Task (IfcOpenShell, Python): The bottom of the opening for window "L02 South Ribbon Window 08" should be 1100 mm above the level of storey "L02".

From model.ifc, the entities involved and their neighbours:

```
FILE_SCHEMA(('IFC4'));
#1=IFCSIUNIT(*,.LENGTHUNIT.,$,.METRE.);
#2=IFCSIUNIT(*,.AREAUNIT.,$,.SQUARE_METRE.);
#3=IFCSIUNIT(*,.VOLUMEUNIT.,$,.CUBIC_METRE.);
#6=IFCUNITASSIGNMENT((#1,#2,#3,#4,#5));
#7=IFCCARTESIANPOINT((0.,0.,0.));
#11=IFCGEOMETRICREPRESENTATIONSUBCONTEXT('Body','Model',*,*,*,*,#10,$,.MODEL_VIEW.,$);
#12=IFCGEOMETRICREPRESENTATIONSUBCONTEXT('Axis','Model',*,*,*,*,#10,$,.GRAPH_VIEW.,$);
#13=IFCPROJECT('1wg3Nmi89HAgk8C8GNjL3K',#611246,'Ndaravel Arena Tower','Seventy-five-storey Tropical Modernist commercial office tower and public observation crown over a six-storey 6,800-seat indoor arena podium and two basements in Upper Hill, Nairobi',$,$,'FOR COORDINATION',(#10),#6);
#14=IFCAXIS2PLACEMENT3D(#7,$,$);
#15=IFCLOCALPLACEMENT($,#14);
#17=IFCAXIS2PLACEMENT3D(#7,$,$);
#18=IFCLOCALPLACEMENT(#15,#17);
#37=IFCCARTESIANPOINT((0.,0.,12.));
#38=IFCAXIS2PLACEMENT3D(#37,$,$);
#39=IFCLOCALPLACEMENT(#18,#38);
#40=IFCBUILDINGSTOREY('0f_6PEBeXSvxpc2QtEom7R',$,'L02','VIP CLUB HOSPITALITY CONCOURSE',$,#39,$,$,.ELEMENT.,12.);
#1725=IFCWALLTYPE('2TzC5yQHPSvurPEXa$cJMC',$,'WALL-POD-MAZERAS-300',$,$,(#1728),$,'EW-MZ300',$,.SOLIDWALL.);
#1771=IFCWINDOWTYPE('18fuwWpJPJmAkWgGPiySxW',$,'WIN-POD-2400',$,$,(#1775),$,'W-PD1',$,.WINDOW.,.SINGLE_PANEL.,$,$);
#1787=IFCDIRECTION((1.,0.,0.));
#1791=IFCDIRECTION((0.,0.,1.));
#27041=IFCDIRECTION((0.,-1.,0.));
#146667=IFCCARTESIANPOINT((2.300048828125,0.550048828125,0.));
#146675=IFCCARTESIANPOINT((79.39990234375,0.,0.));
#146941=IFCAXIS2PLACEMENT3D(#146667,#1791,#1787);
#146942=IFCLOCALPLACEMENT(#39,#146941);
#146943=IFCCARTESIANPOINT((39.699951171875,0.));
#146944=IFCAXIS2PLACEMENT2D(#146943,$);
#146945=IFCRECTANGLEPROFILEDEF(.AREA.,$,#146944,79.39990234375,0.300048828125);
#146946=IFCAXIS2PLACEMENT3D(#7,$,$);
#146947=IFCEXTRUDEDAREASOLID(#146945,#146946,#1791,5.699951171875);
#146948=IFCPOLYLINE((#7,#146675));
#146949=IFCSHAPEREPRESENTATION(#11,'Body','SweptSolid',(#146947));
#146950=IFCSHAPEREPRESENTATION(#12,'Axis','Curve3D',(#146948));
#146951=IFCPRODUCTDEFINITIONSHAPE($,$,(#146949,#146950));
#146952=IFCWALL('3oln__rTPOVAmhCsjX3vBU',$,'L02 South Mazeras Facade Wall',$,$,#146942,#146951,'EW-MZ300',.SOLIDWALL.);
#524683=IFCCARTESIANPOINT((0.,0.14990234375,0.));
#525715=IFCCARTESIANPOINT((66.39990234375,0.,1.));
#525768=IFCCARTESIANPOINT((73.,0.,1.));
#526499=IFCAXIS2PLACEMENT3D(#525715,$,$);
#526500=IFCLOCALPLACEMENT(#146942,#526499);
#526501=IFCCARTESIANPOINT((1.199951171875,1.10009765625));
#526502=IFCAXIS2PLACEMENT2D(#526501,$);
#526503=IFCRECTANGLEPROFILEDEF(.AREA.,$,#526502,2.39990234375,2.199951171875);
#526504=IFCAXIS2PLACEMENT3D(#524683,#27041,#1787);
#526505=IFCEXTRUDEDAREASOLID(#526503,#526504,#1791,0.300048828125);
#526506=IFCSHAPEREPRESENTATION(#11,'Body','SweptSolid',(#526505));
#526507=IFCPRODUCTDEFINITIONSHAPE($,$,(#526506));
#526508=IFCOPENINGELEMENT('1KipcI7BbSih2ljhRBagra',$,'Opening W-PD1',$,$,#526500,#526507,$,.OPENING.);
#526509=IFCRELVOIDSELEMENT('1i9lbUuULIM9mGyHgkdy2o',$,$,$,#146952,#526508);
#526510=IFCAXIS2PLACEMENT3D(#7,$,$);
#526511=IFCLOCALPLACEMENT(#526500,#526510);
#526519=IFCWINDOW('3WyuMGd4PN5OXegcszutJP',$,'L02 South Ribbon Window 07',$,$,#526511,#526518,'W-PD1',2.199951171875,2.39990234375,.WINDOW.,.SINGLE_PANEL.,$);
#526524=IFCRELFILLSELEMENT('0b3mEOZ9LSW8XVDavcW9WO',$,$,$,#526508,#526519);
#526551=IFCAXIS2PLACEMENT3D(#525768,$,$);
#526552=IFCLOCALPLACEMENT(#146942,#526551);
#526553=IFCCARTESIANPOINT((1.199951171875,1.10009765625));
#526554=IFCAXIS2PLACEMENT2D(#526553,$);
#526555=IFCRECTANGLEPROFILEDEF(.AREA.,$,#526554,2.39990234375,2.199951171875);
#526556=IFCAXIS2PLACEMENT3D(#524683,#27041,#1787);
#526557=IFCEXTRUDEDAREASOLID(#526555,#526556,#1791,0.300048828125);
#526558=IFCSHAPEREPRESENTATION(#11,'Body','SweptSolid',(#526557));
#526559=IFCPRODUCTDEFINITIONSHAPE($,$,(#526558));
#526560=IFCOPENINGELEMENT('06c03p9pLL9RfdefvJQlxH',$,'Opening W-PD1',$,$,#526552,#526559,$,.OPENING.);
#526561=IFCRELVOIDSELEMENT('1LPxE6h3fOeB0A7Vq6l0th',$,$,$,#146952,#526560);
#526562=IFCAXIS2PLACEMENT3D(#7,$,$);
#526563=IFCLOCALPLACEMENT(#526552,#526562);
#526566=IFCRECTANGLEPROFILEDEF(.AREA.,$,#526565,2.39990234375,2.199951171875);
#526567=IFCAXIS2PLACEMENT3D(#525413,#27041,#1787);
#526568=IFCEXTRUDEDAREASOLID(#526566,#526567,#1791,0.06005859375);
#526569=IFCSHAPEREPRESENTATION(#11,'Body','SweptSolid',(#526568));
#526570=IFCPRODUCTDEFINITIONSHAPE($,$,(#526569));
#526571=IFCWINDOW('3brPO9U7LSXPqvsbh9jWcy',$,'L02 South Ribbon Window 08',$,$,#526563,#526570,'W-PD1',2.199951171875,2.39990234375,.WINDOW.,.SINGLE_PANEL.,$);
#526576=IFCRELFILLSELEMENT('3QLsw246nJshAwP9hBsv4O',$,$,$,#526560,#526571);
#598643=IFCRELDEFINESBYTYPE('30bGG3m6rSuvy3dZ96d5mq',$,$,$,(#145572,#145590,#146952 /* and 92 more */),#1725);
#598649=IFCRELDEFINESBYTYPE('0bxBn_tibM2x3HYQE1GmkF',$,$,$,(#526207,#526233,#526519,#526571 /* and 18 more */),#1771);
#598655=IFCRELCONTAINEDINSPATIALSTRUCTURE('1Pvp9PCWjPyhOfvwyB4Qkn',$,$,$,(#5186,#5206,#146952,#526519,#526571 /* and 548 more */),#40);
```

```python
import numpy as np
import ifcopenshell
import ifcopenshell.api.geometry
import ifcopenshell.geom
import ifcopenshell.util.element
import ifcopenshell.util.placement
import ifcopenshell.util.shape
import ifcopenshell.util.unit

model = ifcopenshell.open("model.ifc")
unit_scale = ifcopenshell.util.unit.calculate_unit_scale(model)

window = model.by_guid("3brPO9U7LSXPqvsbh9jWcy")
opening = window.FillsVoids[0].RelatingOpeningElement
storey = ifcopenshell.util.element.get_container(window, ifc_class="IfcBuildingStorey")
level = ifcopenshell.util.placement.get_local_placement(storey.ObjectPlacement)[2, 3]

# The opening's origin need not be at the sill, so measure its lowest point.
shape = ifcopenshell.geom.create_shape(ifcopenshell.geom.settings(), opening)
bottom = ifcopenshell.util.shape.get_shape_bottom_elevation(shape, shape.geometry) / unit_scale
dz = level + 1.1 - bottom

shift = np.array([0.0, 0.0, dz])
# The window is placed relative to its opening, so it follows when the opening moves.
matrix = ifcopenshell.util.placement.get_local_placement(opening.ObjectPlacement)
matrix[:3, 3] += shift
ifcopenshell.api.geometry.edit_object_placement(
    model, product=opening, matrix=matrix, is_si=False, should_transform_children=True
)

print(f"moved by {dz * unit_scale:+.3f} m")

model.write("model_rev.ifc")
```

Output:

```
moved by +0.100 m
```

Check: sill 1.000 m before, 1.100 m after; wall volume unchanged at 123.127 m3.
